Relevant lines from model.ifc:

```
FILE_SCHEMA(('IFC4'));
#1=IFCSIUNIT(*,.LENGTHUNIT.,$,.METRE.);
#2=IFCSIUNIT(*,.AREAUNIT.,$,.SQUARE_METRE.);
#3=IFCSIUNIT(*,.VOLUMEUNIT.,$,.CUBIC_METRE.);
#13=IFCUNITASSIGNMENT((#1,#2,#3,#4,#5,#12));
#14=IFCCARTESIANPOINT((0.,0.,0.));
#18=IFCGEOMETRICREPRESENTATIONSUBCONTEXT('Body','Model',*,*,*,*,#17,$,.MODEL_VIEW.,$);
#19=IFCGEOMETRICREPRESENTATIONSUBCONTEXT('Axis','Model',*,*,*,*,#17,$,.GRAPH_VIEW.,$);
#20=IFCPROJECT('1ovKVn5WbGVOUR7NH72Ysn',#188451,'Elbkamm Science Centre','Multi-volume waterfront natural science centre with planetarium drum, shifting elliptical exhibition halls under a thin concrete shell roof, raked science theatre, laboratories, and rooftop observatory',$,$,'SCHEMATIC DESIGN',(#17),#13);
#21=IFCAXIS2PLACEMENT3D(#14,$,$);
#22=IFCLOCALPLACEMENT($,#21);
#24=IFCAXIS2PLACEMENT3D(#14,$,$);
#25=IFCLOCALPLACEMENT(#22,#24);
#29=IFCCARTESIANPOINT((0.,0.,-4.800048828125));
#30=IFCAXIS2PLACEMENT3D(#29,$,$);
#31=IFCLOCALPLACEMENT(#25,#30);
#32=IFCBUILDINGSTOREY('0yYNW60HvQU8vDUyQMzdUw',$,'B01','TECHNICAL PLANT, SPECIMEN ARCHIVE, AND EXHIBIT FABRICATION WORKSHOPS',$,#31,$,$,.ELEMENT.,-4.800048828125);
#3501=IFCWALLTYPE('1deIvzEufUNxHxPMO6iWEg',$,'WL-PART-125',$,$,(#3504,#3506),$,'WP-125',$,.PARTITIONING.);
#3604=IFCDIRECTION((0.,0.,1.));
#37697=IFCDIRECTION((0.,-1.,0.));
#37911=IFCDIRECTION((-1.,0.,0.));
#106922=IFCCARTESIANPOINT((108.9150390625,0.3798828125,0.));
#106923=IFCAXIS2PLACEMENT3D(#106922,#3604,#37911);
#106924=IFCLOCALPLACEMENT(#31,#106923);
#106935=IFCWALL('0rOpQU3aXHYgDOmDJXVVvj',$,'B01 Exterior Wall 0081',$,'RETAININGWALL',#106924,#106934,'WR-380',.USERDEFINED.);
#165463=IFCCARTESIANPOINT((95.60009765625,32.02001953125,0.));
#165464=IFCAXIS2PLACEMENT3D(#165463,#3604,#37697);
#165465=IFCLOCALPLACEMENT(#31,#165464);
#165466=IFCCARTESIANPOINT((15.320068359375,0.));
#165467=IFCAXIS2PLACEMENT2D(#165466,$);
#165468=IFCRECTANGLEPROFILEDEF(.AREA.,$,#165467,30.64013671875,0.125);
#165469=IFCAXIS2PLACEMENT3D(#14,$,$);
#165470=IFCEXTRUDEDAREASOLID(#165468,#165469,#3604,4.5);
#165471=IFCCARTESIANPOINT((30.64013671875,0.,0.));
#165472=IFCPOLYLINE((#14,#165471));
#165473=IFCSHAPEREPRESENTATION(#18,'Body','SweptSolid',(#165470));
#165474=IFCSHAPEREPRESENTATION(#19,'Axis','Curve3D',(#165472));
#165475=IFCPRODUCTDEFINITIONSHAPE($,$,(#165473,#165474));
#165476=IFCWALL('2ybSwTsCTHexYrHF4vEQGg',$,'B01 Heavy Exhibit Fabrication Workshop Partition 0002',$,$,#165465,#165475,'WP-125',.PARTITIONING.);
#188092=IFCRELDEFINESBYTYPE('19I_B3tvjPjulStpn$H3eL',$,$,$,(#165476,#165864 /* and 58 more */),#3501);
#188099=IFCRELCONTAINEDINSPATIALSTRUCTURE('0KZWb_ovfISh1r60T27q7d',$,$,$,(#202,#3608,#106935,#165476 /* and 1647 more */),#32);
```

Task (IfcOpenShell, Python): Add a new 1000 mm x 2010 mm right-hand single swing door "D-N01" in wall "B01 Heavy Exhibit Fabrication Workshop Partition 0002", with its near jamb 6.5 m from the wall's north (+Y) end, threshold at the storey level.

```python
import numpy as np
import ifcopenshell
import ifcopenshell.api.feature
import ifcopenshell.api.geometry
import ifcopenshell.api.root
import ifcopenshell.api.spatial
import ifcopenshell.geom
import ifcopenshell.util.element
import ifcopenshell.util.placement
import ifcopenshell.util.representation
import ifcopenshell.util.shape
import ifcopenshell.util.unit

model = ifcopenshell.open("model.ifc")
unit_scale = ifcopenshell.util.unit.calculate_unit_scale(model)
settings = ifcopenshell.geom.settings()


def volume(element):
    """Net volume in cubic metres, openings subtracted."""
    shape = ifcopenshell.geom.create_shape(settings, element)
    return ifcopenshell.util.shape.get_volume(shape.geometry)


wall = model.by_id(165476)
storey = ifcopenshell.util.element.get_container(wall, ifc_class="IfcBuildingStorey")
context = ifcopenshell.util.representation.get_context(model, "Model", "Body", "MODEL_VIEW")
before = volume(wall)

width, height, from_end, sill = 1, 2.01, 6.5, 0.0  # metres

# The wall runs along its own X axis, and the end named is its -X end.
wall_shape = ifcopenshell.geom.create_shape(settings, wall)
x, y, z = ifcopenshell.util.shape.get_vertices(wall_shape.geometry).T
start = x.min() + from_end
face, thickness = float(y.min()), float(y.max() - y.min())
wall_matrix = ifcopenshell.util.placement.get_local_placement(wall.ObjectPlacement)
level = ifcopenshell.util.placement.get_local_placement(storey.ObjectPlacement)[2, 3]


def in_wall(x, y):
    """Placement at x, y metres in the wall's axes, at sill height."""
    matrix = wall_matrix.copy()
    matrix[:, 3] = wall_matrix @ np.array([x / unit_scale, y / unit_scale, 0.0, 1.0])
    matrix[2, 3] = level + sill / unit_scale
    return matrix


# Opening: a box that overshoots both wall faces by 50 mm.
opening = ifcopenshell.api.root.create_entity(model, ifc_class="IfcOpeningElement", predefined_type="OPENING")
box = ifcopenshell.api.geometry.add_wall_representation(
    model, context=context, length=width, height=height, thickness=thickness + 0.1
)
ifcopenshell.api.geometry.assign_representation(model, product=opening, representation=box)
ifcopenshell.api.geometry.edit_object_placement(model, product=opening, matrix=in_wall(start, face - 0.05), is_si=False)
ifcopenshell.api.feature.add_feature(model, feature=opening, element=wall)

door = ifcopenshell.api.root.create_entity(model, ifc_class="IfcDoor", name="D-N01", predefined_type="DOOR")
door.OverallWidth, door.OverallHeight = width / unit_scale, height / unit_scale
door.OperationType = "SINGLE_SWING_RIGHT"
body = ifcopenshell.api.geometry.add_door_representation(
    model,
    context=context,
    overall_width=door.OverallWidth,
    overall_height=door.OverallHeight,
    operation_type="SINGLE_SWING_RIGHT",
    lining_properties={"LiningDepth": thickness / unit_scale, "ThresholdDepth": thickness / unit_scale},
)
ifcopenshell.api.geometry.assign_representation(model, product=door, representation=body)
ifcopenshell.api.spatial.assign_container(model, products=[door], relating_structure=storey)
ifcopenshell.api.feature.add_filling(model, opening=opening, element=door)

# The lining spans the wall, so the door starts at the wall face.
ifcopenshell.api.geometry.edit_object_placement(model, product=door, matrix=in_wall(start, face), is_si=False)

after = volume(wall)

print(f"wall volume {before:.3f} -> {after:.3f} m3")

model.write("model_v2.ifc")
```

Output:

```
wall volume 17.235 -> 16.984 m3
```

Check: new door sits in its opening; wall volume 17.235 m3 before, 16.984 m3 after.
